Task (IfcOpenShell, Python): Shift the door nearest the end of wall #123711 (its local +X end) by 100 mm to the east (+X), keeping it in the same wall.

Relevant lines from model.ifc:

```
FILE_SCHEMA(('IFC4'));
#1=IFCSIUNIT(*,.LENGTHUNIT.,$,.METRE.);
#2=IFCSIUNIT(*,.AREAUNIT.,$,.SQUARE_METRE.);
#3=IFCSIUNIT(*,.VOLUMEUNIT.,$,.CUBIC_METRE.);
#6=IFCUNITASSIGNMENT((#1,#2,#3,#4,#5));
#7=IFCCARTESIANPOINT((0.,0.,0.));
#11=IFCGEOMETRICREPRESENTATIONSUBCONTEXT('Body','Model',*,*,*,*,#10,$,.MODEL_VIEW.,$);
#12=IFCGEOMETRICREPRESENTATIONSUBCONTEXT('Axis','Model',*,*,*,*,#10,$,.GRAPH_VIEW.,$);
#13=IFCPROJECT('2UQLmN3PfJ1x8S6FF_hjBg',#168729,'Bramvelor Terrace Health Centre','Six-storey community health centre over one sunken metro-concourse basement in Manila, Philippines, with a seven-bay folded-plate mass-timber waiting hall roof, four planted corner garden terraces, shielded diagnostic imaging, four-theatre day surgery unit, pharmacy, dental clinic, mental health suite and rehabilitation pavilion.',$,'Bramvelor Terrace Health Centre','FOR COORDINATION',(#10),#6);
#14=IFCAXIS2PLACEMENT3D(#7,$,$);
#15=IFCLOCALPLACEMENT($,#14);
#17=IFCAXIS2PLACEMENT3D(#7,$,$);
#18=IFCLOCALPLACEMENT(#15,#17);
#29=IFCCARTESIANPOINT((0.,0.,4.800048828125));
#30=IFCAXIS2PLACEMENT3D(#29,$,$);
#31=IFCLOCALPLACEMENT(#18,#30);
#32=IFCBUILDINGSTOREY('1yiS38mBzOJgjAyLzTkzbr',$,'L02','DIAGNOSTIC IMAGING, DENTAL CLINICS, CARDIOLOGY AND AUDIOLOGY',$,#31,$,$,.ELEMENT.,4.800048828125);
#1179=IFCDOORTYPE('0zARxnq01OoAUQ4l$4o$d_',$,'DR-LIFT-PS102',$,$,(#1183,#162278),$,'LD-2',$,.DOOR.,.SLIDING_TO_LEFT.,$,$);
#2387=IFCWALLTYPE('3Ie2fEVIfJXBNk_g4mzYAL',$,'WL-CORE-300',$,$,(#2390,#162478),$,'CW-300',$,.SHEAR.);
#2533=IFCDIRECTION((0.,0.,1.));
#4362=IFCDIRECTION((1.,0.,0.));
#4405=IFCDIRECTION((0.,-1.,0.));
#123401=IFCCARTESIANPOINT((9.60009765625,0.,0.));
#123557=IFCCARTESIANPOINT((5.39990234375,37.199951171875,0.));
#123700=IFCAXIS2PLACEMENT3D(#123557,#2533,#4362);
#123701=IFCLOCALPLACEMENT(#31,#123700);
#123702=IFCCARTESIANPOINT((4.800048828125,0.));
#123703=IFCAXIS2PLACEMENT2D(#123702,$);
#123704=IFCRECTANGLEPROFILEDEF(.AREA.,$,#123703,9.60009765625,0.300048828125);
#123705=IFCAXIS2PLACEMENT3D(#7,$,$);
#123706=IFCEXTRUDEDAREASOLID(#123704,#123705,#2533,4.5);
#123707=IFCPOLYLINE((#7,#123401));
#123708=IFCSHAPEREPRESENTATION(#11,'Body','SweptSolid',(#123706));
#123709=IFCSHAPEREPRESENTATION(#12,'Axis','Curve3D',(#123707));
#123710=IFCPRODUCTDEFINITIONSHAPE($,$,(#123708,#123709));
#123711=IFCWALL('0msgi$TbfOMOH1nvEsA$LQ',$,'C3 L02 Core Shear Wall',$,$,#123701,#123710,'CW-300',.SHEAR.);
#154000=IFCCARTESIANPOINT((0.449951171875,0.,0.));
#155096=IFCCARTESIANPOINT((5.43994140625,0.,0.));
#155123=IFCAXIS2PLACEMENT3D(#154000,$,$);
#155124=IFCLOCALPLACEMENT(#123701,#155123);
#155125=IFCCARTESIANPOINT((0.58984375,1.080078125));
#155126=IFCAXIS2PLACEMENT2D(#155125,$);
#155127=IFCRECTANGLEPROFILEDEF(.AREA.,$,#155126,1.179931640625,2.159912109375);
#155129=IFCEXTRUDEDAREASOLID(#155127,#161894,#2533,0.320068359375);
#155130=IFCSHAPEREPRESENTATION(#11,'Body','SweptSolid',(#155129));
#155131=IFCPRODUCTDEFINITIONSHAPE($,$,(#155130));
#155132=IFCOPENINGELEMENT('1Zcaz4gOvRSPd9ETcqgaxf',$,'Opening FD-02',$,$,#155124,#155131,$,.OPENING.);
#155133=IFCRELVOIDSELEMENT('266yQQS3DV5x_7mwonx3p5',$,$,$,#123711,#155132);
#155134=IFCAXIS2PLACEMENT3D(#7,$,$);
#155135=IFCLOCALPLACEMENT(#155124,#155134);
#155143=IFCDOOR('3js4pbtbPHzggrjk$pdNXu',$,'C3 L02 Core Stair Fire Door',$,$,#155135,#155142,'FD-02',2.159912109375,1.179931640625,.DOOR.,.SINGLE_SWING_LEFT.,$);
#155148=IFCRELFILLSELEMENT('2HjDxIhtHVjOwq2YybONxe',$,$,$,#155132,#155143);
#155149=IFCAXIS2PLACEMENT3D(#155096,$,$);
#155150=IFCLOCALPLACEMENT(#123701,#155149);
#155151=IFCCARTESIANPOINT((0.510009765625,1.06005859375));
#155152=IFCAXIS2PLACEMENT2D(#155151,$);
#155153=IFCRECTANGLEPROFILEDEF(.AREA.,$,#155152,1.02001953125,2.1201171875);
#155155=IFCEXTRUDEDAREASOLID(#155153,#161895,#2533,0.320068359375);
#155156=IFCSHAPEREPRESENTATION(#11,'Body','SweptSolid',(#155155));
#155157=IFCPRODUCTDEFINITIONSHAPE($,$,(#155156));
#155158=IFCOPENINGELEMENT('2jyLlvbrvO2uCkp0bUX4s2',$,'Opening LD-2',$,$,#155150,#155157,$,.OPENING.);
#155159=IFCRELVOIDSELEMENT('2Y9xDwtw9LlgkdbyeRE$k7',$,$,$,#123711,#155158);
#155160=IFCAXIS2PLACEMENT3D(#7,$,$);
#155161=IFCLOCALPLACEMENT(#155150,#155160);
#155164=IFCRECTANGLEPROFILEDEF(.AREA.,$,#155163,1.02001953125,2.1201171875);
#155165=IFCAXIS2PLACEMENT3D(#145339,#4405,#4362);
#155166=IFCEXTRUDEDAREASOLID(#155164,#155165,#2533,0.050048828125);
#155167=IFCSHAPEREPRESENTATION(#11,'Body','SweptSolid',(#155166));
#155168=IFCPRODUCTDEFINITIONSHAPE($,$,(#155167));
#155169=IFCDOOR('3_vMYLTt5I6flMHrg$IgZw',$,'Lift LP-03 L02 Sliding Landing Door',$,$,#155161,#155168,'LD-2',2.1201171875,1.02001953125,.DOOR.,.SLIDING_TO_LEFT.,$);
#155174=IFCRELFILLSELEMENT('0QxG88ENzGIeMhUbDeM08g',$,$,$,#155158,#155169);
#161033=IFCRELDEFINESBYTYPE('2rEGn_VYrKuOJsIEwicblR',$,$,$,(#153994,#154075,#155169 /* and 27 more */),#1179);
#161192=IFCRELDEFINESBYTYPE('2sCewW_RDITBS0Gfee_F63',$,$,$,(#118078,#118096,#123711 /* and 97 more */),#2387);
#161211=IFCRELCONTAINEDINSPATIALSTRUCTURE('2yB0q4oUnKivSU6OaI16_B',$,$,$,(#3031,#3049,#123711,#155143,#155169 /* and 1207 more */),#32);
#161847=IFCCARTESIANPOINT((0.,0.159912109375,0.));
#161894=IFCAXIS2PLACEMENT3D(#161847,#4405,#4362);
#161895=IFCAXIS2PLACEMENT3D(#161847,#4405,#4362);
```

```python
import ifcopenshell
import ifcopenshell.api.geometry
import ifcopenshell.util.placement

model = ifcopenshell.open("model.ifc")

door = model.by_id(155169)
opening = door.FillsVoids[0].RelatingOpeningElement
wall = opening.VoidsElements[0].RelatingBuildingElement

wall_matrix = ifcopenshell.util.placement.get_local_placement(wall.ObjectPlacement)
shift = wall_matrix[:3, 0] * 0.1
before = ifcopenshell.util.placement.get_local_placement(door.ObjectPlacement)[:3, 3].copy()

# The door is placed relative to its opening, so it follows when the opening moves.
matrix = ifcopenshell.util.placement.get_local_placement(opening.ObjectPlacement)
matrix[:3, 3] += shift
ifcopenshell.api.geometry.edit_object_placement(
    model, product=opening, matrix=matrix, is_si=False, should_transform_children=True
)

after = ifcopenshell.util.placement.get_local_placement(door.ObjectPlacement)[:3, 3]
print("door moved by", (after - before).round(3) + 0.0)

model.write("model_updated.ifc")
```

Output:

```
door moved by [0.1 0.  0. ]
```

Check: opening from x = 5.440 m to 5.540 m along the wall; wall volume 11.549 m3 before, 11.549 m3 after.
